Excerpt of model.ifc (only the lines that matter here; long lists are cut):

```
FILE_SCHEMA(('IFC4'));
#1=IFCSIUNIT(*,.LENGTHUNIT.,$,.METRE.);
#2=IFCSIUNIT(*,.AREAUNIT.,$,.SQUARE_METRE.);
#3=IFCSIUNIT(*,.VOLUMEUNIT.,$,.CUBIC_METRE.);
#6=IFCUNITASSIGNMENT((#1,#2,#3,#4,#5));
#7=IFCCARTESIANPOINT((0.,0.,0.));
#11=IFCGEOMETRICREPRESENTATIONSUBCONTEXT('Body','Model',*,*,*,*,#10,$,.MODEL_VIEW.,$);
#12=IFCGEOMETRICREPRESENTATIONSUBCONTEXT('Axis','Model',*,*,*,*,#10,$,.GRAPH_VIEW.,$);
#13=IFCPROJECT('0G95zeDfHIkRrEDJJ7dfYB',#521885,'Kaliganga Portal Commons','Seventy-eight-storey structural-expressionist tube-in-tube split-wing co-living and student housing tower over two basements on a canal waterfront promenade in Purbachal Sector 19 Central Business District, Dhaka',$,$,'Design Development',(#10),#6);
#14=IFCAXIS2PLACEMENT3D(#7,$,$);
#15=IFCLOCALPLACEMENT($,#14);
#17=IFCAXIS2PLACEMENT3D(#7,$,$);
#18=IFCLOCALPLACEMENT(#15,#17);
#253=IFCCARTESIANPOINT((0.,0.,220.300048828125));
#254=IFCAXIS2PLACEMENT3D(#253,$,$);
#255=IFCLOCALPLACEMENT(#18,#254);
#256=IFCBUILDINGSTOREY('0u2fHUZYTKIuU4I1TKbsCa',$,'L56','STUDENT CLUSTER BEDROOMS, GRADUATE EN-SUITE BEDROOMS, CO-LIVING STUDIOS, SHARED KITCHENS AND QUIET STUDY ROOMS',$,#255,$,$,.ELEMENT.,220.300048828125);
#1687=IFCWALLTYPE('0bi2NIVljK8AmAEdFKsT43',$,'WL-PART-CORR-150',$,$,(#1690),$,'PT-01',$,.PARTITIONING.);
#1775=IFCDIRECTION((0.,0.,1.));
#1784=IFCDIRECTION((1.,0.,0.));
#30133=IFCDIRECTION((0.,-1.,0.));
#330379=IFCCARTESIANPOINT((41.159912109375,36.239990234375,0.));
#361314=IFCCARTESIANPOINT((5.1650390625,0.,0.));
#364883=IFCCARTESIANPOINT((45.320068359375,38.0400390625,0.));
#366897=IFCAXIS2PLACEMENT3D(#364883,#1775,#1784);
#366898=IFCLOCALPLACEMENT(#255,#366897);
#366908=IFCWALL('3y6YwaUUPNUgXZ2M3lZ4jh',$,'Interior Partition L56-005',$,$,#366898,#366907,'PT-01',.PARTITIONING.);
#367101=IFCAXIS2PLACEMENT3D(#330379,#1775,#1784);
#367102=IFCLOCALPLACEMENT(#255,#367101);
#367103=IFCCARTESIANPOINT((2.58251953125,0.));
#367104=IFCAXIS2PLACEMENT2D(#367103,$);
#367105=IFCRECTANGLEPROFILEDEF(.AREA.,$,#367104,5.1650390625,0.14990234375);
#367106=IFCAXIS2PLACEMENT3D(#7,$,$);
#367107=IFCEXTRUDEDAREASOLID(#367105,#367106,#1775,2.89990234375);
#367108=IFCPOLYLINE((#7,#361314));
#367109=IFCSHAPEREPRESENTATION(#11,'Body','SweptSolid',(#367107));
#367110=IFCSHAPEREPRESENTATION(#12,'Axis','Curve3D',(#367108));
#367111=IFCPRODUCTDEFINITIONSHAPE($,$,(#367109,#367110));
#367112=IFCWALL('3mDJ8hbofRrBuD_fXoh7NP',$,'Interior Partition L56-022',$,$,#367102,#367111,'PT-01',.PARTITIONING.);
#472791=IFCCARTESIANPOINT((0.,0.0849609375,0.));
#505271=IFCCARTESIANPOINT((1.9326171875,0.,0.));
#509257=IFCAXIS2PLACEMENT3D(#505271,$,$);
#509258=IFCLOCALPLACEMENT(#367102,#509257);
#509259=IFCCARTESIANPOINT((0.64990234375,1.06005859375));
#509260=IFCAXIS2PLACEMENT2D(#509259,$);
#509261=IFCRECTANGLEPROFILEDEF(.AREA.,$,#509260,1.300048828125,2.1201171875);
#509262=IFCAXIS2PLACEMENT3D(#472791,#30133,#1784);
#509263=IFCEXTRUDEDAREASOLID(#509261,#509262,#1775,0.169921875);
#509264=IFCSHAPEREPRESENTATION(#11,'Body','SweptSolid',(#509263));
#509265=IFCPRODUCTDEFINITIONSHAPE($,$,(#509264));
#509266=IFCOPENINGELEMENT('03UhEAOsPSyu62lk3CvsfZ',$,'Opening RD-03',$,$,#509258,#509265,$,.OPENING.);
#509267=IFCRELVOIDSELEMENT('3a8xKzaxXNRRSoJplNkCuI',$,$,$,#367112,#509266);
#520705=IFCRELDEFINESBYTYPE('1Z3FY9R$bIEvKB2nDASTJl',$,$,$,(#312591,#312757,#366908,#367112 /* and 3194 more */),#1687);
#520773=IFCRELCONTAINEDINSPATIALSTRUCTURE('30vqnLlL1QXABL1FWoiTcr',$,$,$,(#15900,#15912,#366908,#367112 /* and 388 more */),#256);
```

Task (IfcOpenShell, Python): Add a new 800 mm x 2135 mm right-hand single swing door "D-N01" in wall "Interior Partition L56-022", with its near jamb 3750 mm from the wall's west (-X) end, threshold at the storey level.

```python
import numpy as np
import ifcopenshell
import ifcopenshell.api.feature
import ifcopenshell.api.geometry
import ifcopenshell.api.root
import ifcopenshell.api.spatial
import ifcopenshell.geom
import ifcopenshell.util.element
import ifcopenshell.util.placement
import ifcopenshell.util.representation
import ifcopenshell.util.shape
import ifcopenshell.util.unit

model = ifcopenshell.open("model.ifc")
unit_scale = ifcopenshell.util.unit.calculate_unit_scale(model)
settings = ifcopenshell.geom.settings()


def volume(element):
    """Net volume in cubic metres, openings subtracted."""
    shape = ifcopenshell.geom.create_shape(settings, element)
    return ifcopenshell.util.shape.get_volume(shape.geometry)


wall = model.by_guid("3mDJ8hbofRrBuD_fXoh7NP")
storey = ifcopenshell.util.element.get_container(wall, ifc_class="IfcBuildingStorey")
context = ifcopenshell.util.representation.get_context(model, "Model", "Body", "MODEL_VIEW")
before = volume(wall)

width, height, from_end, sill = 0.8, 2.135, 3.75, 0.0  # metres

# The wall runs along its own X axis, and the end named is its -X end.
wall_shape = ifcopenshell.geom.create_shape(settings, wall)
x, y, z = ifcopenshell.util.shape.get_vertices(wall_shape.geometry).T
start = x.min() + from_end
face, thickness = float(y.min()), float(y.max() - y.min())
wall_matrix = ifcopenshell.util.placement.get_local_placement(wall.ObjectPlacement)
level = ifcopenshell.util.placement.get_local_placement(storey.ObjectPlacement)[2, 3]


def in_wall(x, y):
    """Placement at x, y metres in the wall's axes, at sill height."""
    matrix = wall_matrix.copy()
    matrix[:, 3] = wall_matrix @ np.array([x / unit_scale, y / unit_scale, 0.0, 1.0])
    matrix[2, 3] = level + sill / unit_scale
    return matrix


# Opening: a box that overshoots both wall faces by 50 mm.
opening = ifcopenshell.api.root.create_entity(model, ifc_class="IfcOpeningElement", predefined_type="OPENING")
box = ifcopenshell.api.geometry.add_wall_representation(
    model, context=context, length=width, height=height, thickness=thickness + 0.1
)
ifcopenshell.api.geometry.assign_representation(model, product=opening, representation=box)
ifcopenshell.api.geometry.edit_object_placement(model, product=opening, matrix=in_wall(start, face - 0.05), is_si=False)
ifcopenshell.api.feature.add_feature(model, feature=opening, element=wall)

door = ifcopenshell.api.root.create_entity(model, ifc_class="IfcDoor", name="D-N01", predefined_type="DOOR")
door.OverallWidth, door.OverallHeight = width / unit_scale, height / unit_scale
door.OperationType = "SINGLE_SWING_RIGHT"
body = ifcopenshell.api.geometry.add_door_representation(
    model,
    context=context,
    overall_width=door.OverallWidth,
    overall_height=door.OverallHeight,
    operation_type="SINGLE_SWING_RIGHT",
    lining_properties={"LiningDepth": thickness / unit_scale, "ThresholdDepth": thickness / unit_scale},
)
ifcopenshell.api.geometry.assign_representation(model, product=door, representation=body)
ifcopenshell.api.spatial.assign_container(model, products=[door], relating_structure=storey)
ifcopenshell.api.feature.add_filling(model, opening=opening, element=door)

# The lining spans the wall, so the door starts at the wall face.
ifcopenshell.api.geometry.edit_object_placement(model, product=door, matrix=in_wall(start, face), is_si=False)

after = volume(wall)

print(f"wall volume {before:.3f} -> {after:.3f} m3")

model.write("model_updated.ifc")
```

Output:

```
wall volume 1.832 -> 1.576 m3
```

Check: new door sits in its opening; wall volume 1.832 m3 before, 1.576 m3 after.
